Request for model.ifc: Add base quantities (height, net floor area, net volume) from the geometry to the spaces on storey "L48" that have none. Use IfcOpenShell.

First a look at what the model holds.

```python
import ifcopenshell
import ifcopenshell.util.element
import ifcopenshell.util.unit

model = ifcopenshell.open("model.ifc")
print(model.schema)
for unit_type in ("LENGTHUNIT", "AREAUNIT", "VOLUMEUNIT"):
    print(unit_type, ifcopenshell.util.unit.calculate_unit_scale(model, unit_type))
storey = next(s for s in model.by_type("IfcBuildingStorey") if s.Name == "L48")
spaces = [e for e in ifcopenshell.util.element.get_decomposition(storey) if e.is_a("IfcSpace")]
for e in sorted(spaces, key=lambda e: e.id()):
    print(e.id(), e.is_a(), e.Name, list(ifcopenshell.util.element.get_psets(e, qtos_only=True)), sep=" | ")
```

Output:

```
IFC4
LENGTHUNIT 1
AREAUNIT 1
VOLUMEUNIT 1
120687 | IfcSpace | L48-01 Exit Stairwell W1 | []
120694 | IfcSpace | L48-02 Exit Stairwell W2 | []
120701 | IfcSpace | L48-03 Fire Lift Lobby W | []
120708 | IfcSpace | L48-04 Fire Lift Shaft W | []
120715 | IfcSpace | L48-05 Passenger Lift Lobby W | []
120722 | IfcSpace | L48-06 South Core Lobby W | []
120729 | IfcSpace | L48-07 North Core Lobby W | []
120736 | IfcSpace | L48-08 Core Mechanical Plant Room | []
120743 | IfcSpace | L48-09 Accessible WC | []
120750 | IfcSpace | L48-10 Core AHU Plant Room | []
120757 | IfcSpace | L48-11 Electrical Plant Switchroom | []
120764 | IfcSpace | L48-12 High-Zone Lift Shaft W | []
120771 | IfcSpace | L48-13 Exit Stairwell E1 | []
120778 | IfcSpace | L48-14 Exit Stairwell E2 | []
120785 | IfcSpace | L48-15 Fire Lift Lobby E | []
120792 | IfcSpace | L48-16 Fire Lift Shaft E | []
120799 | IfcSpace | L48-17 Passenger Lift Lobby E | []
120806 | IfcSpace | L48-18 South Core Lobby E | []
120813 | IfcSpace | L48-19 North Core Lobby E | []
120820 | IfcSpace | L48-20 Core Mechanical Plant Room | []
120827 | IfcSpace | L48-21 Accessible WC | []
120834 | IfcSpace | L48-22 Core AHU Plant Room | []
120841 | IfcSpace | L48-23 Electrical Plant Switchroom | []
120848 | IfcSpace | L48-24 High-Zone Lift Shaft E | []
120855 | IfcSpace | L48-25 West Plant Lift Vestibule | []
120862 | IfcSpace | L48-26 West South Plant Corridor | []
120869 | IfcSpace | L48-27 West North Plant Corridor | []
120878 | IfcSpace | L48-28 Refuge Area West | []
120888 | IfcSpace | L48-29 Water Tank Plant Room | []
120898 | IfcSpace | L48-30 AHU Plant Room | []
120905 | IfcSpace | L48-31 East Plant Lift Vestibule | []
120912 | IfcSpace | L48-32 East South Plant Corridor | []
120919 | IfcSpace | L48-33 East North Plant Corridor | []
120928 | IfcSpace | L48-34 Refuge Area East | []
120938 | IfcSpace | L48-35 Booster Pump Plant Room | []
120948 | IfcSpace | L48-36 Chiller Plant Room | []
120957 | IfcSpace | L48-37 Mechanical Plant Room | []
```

```python
import ifcopenshell
import ifcopenshell.api.pset
import ifcopenshell.geom
import ifcopenshell.util.element
import ifcopenshell.util.shape
import ifcopenshell.util.unit

model = ifcopenshell.open("model.ifc")
unit_scale = ifcopenshell.util.unit.calculate_unit_scale(model)
area_scale = ifcopenshell.util.unit.calculate_unit_scale(model, "AREAUNIT")
volume_scale = ifcopenshell.util.unit.calculate_unit_scale(model, "VOLUMEUNIT")
settings = ifcopenshell.geom.settings()

storey = next(s for s in model.by_type("IfcBuildingStorey") if s.Name == "L48")
spaces = [e for e in ifcopenshell.util.element.get_decomposition(storey) if e.is_a("IfcSpace")]

for e in sorted(spaces, key=lambda e: e.id()):
    if ifcopenshell.util.element.get_psets(e, qtos_only=True, should_inherit=False):
        continue
    # Geometry comes back in metres, in the element's own axes.
    shape = ifcopenshell.geom.create_shape(settings, e)
    values = {
        "Height": ifcopenshell.util.shape.get_z(shape.geometry) / unit_scale,
        "NetFloorArea": ifcopenshell.util.shape.get_footprint_area(shape.geometry) / area_scale,
        "NetVolume": ifcopenshell.util.shape.get_volume(shape.geometry) / volume_scale,
    }
    qto = ifcopenshell.api.pset.add_qto(model, product=e, name="Qto_SpaceBaseQuantities")
    ifcopenshell.api.pset.edit_qto(model, qto=qto, properties=values)
    print(e.id(), {k: round(v, 3) for k, v in values.items()})

model.write("model-out.ifc")
```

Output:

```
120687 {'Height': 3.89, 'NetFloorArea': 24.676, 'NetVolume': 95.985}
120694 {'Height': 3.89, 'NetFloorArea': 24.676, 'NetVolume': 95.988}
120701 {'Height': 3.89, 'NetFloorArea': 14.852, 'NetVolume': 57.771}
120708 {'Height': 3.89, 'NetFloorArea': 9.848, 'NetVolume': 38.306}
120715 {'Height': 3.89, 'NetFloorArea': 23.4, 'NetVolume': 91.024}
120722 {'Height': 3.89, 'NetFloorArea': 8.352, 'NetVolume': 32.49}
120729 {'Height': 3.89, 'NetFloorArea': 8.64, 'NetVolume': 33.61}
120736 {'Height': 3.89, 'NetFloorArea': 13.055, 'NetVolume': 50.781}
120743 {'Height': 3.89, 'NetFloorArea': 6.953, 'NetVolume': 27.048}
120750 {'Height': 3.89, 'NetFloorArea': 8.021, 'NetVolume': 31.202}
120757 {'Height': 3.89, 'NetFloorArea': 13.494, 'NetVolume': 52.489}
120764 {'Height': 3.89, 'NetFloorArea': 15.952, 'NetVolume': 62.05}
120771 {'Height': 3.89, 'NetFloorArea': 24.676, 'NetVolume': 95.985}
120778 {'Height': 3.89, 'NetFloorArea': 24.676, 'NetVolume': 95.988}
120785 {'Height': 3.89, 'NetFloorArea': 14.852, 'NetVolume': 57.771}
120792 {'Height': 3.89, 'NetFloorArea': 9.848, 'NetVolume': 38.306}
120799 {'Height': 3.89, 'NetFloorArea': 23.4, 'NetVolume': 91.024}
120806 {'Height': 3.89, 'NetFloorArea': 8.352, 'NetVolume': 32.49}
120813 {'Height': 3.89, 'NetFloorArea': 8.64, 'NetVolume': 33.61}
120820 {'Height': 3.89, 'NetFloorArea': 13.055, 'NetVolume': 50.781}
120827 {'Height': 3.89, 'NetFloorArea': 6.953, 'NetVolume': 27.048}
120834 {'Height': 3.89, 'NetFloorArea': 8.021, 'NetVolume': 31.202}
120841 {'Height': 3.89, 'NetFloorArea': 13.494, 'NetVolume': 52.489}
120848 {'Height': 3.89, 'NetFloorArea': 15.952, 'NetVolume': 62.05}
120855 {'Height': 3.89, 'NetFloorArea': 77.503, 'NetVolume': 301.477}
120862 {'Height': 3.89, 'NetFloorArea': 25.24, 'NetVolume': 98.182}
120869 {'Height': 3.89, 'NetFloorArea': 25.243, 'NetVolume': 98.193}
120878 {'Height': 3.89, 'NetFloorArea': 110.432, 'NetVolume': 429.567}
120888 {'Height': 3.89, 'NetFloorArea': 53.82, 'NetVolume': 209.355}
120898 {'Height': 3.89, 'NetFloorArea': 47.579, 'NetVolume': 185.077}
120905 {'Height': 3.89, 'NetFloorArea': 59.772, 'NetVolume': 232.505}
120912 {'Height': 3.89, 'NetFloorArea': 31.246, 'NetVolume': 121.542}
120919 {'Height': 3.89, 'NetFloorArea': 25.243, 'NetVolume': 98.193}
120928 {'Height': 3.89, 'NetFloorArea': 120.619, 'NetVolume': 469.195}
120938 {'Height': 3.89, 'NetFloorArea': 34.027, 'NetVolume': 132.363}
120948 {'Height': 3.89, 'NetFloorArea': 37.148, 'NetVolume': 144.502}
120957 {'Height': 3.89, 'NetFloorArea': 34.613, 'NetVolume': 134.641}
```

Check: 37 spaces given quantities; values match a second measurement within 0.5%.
